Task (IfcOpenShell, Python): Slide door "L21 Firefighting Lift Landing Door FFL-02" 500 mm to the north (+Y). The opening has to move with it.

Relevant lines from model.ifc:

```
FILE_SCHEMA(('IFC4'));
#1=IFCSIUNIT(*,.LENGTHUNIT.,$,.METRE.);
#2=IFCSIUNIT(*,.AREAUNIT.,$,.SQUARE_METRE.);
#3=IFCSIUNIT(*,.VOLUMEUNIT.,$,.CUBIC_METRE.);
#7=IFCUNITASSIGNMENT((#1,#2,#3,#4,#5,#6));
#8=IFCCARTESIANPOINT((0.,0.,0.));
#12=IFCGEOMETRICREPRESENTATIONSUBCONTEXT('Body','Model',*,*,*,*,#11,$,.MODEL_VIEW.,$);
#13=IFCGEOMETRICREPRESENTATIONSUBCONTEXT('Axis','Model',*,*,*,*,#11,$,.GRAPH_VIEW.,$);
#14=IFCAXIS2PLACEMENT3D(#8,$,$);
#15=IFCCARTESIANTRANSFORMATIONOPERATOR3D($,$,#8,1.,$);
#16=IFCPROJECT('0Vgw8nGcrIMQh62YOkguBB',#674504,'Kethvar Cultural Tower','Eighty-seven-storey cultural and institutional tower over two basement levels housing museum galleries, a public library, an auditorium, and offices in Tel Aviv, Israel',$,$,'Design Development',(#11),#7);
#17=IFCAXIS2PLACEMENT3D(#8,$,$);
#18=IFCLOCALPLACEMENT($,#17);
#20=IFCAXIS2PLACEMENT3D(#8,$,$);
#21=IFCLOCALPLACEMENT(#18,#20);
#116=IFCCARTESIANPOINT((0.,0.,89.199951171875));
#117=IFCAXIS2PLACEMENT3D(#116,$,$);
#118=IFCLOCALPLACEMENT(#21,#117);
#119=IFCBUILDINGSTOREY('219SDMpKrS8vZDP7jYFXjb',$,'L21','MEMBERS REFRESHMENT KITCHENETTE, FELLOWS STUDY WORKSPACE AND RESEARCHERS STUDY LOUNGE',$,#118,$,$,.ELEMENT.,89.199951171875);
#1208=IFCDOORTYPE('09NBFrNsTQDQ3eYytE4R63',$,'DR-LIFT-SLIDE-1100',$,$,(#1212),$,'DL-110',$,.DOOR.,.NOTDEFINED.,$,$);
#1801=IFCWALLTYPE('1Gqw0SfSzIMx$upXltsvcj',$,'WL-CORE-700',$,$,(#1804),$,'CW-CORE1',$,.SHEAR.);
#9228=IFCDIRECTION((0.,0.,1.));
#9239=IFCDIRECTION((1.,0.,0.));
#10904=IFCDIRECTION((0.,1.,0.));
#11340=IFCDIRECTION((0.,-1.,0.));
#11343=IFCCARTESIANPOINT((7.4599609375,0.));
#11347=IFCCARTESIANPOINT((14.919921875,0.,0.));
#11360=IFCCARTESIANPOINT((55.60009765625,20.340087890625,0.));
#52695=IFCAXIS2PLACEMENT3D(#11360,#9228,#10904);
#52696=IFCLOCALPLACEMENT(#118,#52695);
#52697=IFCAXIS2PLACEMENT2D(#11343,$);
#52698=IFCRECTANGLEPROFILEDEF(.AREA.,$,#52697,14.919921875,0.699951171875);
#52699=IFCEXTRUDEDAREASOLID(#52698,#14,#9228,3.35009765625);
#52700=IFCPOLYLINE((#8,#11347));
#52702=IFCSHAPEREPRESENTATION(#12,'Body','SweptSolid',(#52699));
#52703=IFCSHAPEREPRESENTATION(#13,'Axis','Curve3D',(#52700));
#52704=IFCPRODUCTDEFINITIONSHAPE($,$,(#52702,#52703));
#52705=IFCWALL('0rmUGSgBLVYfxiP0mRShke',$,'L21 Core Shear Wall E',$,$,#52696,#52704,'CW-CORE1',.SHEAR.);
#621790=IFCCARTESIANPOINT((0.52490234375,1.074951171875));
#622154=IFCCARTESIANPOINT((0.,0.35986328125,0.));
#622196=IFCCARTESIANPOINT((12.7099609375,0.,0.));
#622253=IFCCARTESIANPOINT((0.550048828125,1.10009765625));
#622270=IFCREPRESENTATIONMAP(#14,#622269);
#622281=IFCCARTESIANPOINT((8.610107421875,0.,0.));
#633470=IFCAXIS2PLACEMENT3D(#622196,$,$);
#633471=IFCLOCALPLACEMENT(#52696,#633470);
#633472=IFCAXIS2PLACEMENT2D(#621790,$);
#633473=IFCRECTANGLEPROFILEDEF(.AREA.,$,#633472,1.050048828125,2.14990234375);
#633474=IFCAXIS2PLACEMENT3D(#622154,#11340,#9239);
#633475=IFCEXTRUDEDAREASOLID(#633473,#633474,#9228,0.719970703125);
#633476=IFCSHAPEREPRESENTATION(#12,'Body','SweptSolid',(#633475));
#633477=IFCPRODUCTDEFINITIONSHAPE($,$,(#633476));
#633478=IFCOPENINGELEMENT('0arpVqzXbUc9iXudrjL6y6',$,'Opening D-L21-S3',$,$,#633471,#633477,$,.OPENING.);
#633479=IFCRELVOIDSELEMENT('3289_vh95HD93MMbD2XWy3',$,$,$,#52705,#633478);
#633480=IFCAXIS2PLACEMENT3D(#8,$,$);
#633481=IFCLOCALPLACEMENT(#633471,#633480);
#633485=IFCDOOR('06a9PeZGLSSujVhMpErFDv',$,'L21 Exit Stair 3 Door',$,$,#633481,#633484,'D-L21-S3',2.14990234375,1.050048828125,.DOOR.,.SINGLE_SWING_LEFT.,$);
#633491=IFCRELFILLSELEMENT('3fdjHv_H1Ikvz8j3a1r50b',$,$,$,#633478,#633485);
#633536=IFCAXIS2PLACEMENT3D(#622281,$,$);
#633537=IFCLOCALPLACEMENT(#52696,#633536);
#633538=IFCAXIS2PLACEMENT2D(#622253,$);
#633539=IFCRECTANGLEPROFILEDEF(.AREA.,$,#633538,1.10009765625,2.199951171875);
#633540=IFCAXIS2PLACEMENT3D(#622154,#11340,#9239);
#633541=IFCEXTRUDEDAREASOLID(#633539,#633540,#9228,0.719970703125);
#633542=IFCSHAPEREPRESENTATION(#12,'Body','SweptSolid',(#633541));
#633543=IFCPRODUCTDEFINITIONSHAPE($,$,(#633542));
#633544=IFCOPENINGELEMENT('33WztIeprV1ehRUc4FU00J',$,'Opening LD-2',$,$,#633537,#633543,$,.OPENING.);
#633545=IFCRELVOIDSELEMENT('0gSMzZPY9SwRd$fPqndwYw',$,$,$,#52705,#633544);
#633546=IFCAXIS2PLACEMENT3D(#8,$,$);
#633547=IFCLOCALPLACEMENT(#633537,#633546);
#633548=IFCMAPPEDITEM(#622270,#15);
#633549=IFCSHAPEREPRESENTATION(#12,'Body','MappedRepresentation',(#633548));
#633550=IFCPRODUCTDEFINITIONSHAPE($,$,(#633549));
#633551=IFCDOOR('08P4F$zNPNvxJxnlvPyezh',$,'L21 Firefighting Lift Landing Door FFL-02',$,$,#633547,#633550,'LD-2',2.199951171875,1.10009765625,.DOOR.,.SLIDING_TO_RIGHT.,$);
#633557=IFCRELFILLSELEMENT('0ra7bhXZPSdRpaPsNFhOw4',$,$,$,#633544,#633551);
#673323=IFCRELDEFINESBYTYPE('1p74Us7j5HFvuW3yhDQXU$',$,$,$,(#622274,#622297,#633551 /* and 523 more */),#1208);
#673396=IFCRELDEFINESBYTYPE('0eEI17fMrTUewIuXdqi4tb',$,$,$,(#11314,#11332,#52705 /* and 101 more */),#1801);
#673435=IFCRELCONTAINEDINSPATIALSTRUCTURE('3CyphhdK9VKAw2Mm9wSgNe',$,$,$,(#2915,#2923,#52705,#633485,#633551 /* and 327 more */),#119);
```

```python
import ifcopenshell
import ifcopenshell.api.geometry
import ifcopenshell.util.placement
import ifcopenshell.util.unit

model = ifcopenshell.open("model.ifc")
unit_scale = ifcopenshell.util.unit.calculate_unit_scale(model)

door = model.by_id(633551)
opening = door.FillsVoids[0].RelatingOpeningElement
wall = opening.VoidsElements[0].RelatingBuildingElement

wall_matrix = ifcopenshell.util.placement.get_local_placement(wall.ObjectPlacement)
shift = wall_matrix[:3, 0] * 0.5 / unit_scale
before = ifcopenshell.util.placement.get_local_placement(door.ObjectPlacement)[:3, 3].copy()

# The door is placed relative to its opening, so it follows when the opening moves.
matrix = ifcopenshell.util.placement.get_local_placement(opening.ObjectPlacement)
matrix[:3, 3] += shift
ifcopenshell.api.geometry.edit_object_placement(
    model, product=opening, matrix=matrix, is_si=False, should_transform_children=True
)

after = ifcopenshell.util.placement.get_local_placement(door.ObjectPlacement)[:3, 3]
print("door moved by", (after - before).round(3) + 0.0)

model.write("model_edited.ifc")
```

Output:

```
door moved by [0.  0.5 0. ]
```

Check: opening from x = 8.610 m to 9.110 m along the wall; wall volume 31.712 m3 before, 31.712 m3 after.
